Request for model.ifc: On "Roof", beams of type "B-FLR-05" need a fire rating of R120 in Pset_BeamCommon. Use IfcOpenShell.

First a look at what the model holds.

```python
import ifcopenshell
import ifcopenshell.util.element

model = ifcopenshell.open("model.ifc")
print(model.schema)
storey = next(s for s in model.by_type("IfcBuildingStorey") if s.Name == "Roof")
beams = [e for e in ifcopenshell.util.element.get_decomposition(storey) if e.is_a("IfcBeam")]
seen = {}
for e in beams:
    element_type = ifcopenshell.util.element.get_type(e)
    key = (element_type.Name if element_type != e and element_type else None, ifcopenshell.util.element.get_pset(e, "Pset_BeamCommon", "FireRating"))
    seen[key] = seen.get(key, 0) + 1
for (name, value), count in sorted(seen.items(), key=str):
    print(count, "x", name, "|", value)
```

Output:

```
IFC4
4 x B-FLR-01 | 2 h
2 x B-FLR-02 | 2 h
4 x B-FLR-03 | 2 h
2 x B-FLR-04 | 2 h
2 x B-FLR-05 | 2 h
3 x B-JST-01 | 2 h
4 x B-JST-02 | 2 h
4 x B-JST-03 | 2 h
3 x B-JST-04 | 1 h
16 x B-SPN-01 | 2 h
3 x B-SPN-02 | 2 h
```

```python
import ifcopenshell
import ifcopenshell.api.pset
import ifcopenshell.util.element

model = ifcopenshell.open("model.ifc")

storey = next(s for s in model.by_type("IfcBuildingStorey") if s.Name == "Roof")
beams = [e for e in ifcopenshell.util.element.get_decomposition(storey) if e.is_a("IfcBeam")]

count = 0
for e in beams:
    element_type = ifcopenshell.util.element.get_type(e)
    if element_type in (None, e) or element_type.Name != "B-FLR-05":
        continue
    # add_pset returns the element's existing set when there is one.
    pset = ifcopenshell.api.pset.add_pset(model, product=e, name="Pset_BeamCommon")
    ifcopenshell.api.pset.edit_pset(model, pset=pset, properties={"FireRating": "R120"})
    count += 1

print(count, "beams updated")

model.write("model_edited.ifc")
```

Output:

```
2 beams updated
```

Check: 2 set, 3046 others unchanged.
